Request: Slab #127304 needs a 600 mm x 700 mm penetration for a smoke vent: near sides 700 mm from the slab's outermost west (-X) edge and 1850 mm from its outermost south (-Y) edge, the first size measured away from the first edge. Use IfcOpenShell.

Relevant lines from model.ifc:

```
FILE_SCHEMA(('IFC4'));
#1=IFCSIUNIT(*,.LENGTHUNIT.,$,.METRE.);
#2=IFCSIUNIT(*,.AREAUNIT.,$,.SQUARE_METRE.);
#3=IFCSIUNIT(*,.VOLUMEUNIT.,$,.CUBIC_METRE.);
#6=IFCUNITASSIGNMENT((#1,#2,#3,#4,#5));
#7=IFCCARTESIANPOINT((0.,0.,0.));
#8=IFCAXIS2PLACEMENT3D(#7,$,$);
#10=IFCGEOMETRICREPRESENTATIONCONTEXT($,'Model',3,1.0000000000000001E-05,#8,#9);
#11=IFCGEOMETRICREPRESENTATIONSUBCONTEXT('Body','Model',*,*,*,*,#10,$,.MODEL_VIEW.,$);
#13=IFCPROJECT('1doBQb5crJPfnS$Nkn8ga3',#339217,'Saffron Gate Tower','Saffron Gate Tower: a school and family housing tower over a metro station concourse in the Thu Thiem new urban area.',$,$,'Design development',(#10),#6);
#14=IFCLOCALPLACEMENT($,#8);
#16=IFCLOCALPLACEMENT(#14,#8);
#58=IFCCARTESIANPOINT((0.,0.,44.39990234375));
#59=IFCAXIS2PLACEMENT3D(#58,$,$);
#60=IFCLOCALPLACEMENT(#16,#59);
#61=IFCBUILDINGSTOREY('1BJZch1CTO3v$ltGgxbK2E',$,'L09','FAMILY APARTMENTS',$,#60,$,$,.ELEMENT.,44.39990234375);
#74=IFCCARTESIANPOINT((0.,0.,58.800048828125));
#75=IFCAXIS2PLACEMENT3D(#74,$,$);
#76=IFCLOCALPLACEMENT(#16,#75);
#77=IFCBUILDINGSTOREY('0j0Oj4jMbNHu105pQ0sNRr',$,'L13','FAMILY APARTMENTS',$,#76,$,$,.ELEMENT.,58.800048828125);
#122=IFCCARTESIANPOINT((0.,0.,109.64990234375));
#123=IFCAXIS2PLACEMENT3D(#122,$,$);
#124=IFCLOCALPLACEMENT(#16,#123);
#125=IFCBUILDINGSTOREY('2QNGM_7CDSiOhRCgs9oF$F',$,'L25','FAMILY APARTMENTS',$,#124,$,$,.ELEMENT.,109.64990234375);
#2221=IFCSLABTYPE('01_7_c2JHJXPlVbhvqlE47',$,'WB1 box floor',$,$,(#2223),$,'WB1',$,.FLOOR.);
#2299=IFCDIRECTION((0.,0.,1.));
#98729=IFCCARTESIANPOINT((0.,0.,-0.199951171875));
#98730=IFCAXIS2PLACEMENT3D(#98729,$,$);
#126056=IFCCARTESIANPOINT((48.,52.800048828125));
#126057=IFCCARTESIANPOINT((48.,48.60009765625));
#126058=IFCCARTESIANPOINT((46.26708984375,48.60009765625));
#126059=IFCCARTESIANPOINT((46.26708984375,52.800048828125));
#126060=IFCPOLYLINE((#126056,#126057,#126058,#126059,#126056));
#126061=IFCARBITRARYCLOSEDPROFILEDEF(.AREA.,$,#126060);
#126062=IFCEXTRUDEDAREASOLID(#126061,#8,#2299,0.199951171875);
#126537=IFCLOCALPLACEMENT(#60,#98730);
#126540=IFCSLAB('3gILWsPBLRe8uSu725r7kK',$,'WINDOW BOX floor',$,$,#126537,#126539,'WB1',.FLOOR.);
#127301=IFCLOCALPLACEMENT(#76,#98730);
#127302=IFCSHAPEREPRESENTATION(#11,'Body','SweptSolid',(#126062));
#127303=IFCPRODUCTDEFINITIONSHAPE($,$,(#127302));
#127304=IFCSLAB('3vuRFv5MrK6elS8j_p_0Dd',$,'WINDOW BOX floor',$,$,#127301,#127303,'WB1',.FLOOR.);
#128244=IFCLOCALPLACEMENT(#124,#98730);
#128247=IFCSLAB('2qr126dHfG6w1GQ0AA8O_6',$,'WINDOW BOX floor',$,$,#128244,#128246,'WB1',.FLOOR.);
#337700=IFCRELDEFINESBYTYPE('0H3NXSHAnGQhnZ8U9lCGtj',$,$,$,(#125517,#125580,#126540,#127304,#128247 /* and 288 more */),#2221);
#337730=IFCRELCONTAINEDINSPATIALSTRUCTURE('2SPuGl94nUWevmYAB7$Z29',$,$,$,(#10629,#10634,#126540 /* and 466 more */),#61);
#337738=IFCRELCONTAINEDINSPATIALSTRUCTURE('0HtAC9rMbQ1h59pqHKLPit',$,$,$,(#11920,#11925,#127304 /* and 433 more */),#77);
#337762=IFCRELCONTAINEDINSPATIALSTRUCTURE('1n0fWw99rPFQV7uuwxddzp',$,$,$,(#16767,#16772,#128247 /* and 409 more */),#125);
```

```python
import numpy as np
import ifcopenshell
import ifcopenshell.api.feature
import ifcopenshell.api.geometry
import ifcopenshell.api.root
import ifcopenshell.geom
import ifcopenshell.util.placement
import ifcopenshell.util.representation
import ifcopenshell.util.shape
import ifcopenshell.util.unit

model = ifcopenshell.open("model.ifc")
unit_scale = ifcopenshell.util.unit.calculate_unit_scale(model)
settings = ifcopenshell.geom.settings()


def volume(element):
    """Net volume in cubic metres, openings subtracted."""
    shape = ifcopenshell.geom.create_shape(settings, element)
    return ifcopenshell.util.shape.get_volume(shape.geometry)


slab = model.by_guid("3vuRFv5MrK6elS8j_p_0Dd")
before = volume(slab)

# Extent in the slab's own axes, in metres. The edges named are its -X and -Y sides.
slab_shape = ifcopenshell.geom.create_shape(settings, slab)
vertices = ifcopenshell.util.shape.get_vertices(slab_shape.geometry)
x_min, y_min, bottom = vertices.min(axis=0)
top = vertices[:, 2].max()

opening = ifcopenshell.api.root.create_entity(model, ifc_class="IfcOpeningElement", name="Smoke vent opening", predefined_type="OPENING")
context = ifcopenshell.util.representation.get_context(model, "Model", "Body", "MODEL_VIEW")
width, depth = 0.6, 0.7
outline = [(0.0, 0.0), (width, 0.0), (width, depth), (0.0, depth), (0.0, 0.0)]
# Overshoot both faces by 50 mm so the cut is clean.
shape = ifcopenshell.api.geometry.add_slab_representation(
    model, context=context, depth=top - bottom + 0.1, polyline=outline
)
ifcopenshell.api.geometry.assign_representation(model, product=opening, representation=shape)

matrix = ifcopenshell.util.placement.get_local_placement(slab.ObjectPlacement)
matrix[:, 3] = matrix @ np.append(np.array([x_min + 0.7, y_min + 1.85, bottom - 0.05]) / unit_scale, 1.0)
ifcopenshell.api.geometry.edit_object_placement(model, product=opening, matrix=matrix, is_si=False)
ifcopenshell.api.feature.add_feature(model, feature=opening, element=slab)

after = volume(slab)

print(f"slab volume {before:.3f} -> {after:.3f} m3")

model.write("model_updated.ifc")
```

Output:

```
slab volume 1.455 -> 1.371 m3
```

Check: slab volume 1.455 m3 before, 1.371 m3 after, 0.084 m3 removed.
